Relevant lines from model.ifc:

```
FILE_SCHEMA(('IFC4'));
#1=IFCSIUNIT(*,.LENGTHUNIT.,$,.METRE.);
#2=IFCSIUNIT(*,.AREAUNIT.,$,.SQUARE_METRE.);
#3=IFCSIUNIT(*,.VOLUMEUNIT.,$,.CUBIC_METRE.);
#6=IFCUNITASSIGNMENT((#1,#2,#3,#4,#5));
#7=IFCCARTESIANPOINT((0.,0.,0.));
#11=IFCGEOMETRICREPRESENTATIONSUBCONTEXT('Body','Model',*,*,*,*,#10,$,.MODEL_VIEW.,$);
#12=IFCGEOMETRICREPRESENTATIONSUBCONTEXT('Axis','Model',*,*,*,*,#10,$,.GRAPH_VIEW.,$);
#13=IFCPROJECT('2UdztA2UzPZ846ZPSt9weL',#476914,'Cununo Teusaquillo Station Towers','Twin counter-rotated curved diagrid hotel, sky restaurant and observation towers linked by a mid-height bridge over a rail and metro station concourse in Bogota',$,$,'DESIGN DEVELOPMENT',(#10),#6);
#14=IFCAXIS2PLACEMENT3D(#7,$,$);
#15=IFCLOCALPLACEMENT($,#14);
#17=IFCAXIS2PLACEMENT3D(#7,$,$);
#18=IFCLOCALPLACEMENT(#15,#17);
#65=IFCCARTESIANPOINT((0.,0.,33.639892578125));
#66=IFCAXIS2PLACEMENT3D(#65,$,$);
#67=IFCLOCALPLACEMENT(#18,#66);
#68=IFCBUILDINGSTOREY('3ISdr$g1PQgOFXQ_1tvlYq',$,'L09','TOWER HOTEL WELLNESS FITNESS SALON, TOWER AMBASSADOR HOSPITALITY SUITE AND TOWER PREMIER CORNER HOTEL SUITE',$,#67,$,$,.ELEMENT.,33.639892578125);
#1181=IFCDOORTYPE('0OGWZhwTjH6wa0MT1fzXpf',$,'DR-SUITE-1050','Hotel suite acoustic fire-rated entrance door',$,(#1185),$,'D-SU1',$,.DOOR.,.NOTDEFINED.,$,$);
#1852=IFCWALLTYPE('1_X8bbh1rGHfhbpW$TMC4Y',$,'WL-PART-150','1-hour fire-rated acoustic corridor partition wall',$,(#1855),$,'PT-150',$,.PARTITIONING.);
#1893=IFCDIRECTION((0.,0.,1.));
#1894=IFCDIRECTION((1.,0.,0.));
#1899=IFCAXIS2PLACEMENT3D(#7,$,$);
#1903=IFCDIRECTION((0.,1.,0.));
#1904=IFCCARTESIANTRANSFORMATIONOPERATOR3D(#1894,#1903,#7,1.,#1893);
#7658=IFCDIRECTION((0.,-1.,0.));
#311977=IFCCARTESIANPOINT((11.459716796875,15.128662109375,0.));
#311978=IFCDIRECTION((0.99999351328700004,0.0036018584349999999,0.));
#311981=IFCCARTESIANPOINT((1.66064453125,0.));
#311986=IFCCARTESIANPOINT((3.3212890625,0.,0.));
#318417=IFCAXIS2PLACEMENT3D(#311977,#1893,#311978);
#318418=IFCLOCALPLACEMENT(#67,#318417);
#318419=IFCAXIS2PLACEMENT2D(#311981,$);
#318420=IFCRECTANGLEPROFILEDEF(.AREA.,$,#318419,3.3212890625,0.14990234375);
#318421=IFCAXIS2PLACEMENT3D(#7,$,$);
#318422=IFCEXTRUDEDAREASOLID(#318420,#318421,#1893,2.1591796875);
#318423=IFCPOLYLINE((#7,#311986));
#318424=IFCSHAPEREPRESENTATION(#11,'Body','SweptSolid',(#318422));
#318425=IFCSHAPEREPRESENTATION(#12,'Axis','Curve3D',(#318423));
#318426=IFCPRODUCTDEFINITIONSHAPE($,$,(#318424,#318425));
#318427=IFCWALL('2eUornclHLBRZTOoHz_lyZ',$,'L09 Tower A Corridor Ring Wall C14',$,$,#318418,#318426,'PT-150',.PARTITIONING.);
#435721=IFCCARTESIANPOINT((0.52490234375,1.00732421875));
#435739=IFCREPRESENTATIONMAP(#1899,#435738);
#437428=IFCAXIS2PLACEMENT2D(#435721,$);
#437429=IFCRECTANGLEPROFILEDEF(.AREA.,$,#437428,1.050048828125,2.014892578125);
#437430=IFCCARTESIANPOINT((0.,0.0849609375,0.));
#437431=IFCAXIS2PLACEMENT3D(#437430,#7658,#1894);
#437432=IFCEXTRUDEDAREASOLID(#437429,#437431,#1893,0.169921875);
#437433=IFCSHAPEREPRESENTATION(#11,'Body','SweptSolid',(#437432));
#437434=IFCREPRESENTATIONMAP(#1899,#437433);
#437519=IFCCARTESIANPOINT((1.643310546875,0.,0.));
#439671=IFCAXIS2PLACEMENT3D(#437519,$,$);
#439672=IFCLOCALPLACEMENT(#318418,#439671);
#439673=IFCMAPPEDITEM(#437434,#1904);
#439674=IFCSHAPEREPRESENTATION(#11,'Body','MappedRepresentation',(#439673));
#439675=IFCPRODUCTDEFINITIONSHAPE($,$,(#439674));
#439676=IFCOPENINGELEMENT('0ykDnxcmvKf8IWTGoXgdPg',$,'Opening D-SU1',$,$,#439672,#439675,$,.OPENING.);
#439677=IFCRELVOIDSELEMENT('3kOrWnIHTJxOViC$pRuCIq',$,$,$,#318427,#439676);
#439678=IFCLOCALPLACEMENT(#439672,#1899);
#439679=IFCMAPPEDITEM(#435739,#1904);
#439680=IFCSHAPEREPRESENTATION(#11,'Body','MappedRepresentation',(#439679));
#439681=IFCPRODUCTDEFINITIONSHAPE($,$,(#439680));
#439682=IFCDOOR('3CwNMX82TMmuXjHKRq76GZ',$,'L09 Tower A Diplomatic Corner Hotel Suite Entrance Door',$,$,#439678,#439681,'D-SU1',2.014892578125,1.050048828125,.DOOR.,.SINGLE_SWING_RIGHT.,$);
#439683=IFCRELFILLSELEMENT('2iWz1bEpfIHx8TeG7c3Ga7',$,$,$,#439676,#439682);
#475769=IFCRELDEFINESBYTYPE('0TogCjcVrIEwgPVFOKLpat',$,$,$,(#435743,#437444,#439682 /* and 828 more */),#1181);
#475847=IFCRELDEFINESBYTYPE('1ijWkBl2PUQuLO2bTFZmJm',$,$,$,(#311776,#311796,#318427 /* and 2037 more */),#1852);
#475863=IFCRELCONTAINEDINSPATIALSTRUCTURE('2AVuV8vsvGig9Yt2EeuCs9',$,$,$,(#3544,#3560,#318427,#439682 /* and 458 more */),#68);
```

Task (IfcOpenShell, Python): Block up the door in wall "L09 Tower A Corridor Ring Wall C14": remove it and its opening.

```python
import ifcopenshell
import ifcopenshell.api.feature
import ifcopenshell.api.root
import ifcopenshell.geom
import ifcopenshell.util.shape

model = ifcopenshell.open("model.ifc")
settings = ifcopenshell.geom.settings()


def volume(element):
    """Net volume in cubic metres, openings subtracted."""
    shape = ifcopenshell.geom.create_shape(settings, element)
    return ifcopenshell.util.shape.get_volume(shape.geometry)


door = model.by_guid("3CwNMX82TMmuXjHKRq76GZ")
opening = door.FillsVoids[0].RelatingOpeningElement
wall = opening.VoidsElements[0].RelatingBuildingElement
before = volume(wall)

ifcopenshell.api.root.remove_product(model, product=door)
ifcopenshell.api.feature.remove_feature(model, feature=opening)

after = volume(wall)

print(f"wall volume {before:.3f} -> {after:.3f} m3")

model.write("model_updated.ifc")
```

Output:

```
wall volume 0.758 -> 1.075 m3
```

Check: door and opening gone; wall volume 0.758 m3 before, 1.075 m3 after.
